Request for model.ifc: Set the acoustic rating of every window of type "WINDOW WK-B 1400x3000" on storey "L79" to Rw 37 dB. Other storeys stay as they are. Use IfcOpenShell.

First a look at what the model holds.

```python
import ifcopenshell
import ifcopenshell.util.element

model = ifcopenshell.open("model.ifc")
print(model.schema)
storey = next(s for s in model.by_type("IfcBuildingStorey") if s.Name == "L79")
windows = [e for e in ifcopenshell.util.element.get_decomposition(storey) if e.is_a("IfcWindow")]
seen = {}
for e in windows:
    element_type = ifcopenshell.util.element.get_type(e)
    key = (element_type.Name if element_type != e and element_type else None, ifcopenshell.util.element.get_pset(e, "Pset_WindowCommon", "AcousticRating"))
    seen[key] = seen.get(key, 0) + 1
for (name, value), count in sorted(seen.items(), key=str):
    print(count, "x", name, "|", value)
```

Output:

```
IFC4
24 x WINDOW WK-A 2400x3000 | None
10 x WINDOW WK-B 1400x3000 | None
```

```python
import ifcopenshell
import ifcopenshell.api.pset
import ifcopenshell.util.element

model = ifcopenshell.open("model.ifc")

storey = next(s for s in model.by_type("IfcBuildingStorey") if s.Name == "L79")
windows = [e for e in ifcopenshell.util.element.get_decomposition(storey) if e.is_a("IfcWindow")]

count = 0
for e in windows:
    element_type = ifcopenshell.util.element.get_type(e)
    if element_type in (None, e) or element_type.Name != "WINDOW WK-B 1400x3000":
        continue
    found = ifcopenshell.util.element.get_pset(e, "Pset_WindowCommon", should_inherit=False)
    if found:
        pset = model.by_id(found["id"])
        if len(ifcopenshell.util.element.get_elements_by_pset(pset)) > 1:
            pset = ifcopenshell.api.pset.unshare_pset(model, products=[e], pset=pset)[0]
    else:
        pset = ifcopenshell.api.pset.add_pset(model, product=e, name="Pset_WindowCommon")
    ifcopenshell.api.pset.edit_pset(model, pset=pset, properties={"AcousticRating": "Rw 37 dB"})
    count += 1

print(count, "windows updated")

model.write("model-out.ifc")
```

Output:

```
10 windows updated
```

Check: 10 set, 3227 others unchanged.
